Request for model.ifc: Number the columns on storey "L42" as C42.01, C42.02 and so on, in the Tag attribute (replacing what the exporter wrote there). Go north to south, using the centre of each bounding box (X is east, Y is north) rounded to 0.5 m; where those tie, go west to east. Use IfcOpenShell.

First a look at what the model holds.

```python
import ifcopenshell
import ifcopenshell.util.element
import ifcopenshell.util.placement

model = ifcopenshell.open("model.ifc")
print(model.schema)
storey = next(s for s in model.by_type("IfcBuildingStorey") if s.Name == "L42")
columns = [e for e in ifcopenshell.util.element.get_decomposition(storey) if e.is_a("IfcColumn")]
for e in sorted(columns, key=lambda e: e.id()):
    origin = ifcopenshell.util.placement.get_local_placement(e.ObjectPlacement)[:3, 3]
    print(e.id(), e.Tag, e.Name, origin.round(2) + 0.0, sep=" | ")
```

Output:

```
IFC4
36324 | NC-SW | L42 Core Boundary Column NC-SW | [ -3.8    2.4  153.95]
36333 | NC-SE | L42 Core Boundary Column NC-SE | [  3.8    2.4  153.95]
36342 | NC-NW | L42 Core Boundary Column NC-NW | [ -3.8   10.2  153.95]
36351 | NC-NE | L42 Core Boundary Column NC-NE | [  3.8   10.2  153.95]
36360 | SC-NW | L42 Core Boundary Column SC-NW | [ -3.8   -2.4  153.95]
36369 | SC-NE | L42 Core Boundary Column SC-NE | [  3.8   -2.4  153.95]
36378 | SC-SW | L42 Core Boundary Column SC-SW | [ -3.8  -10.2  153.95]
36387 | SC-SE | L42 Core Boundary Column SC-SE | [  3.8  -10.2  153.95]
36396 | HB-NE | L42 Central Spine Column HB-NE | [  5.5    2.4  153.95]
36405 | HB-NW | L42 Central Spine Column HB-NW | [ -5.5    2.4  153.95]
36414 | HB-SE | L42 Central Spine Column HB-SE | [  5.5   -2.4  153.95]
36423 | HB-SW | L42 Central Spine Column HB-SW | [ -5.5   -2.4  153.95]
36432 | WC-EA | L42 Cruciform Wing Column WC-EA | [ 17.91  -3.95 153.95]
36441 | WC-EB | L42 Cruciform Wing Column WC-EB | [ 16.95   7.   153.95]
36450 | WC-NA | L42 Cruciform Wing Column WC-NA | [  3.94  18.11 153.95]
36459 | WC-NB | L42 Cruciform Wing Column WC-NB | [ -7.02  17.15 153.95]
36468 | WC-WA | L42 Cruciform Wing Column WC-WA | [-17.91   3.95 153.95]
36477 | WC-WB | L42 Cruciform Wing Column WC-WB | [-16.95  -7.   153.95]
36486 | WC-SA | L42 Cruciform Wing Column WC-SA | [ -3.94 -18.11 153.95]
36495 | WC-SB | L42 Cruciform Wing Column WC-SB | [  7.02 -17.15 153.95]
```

```python
import ifcopenshell
import ifcopenshell.geom
import ifcopenshell.util.element
import ifcopenshell.util.shape

model = ifcopenshell.open("model.ifc")
settings = ifcopenshell.geom.settings()
settings.set("use-world-coords", True)


def centre(element):
    shape = ifcopenshell.geom.create_shape(settings, element)
    return ifcopenshell.util.shape.get_bbox_centroid(shape.geometry)


storey = next(s for s in model.by_type("IfcBuildingStorey") if s.Name == "L42")
columns = [e for e in ifcopenshell.util.element.get_decomposition(storey) if e.is_a("IfcColumn")]

# Insertion points can sit at a corner or the storey origin, so sort by the geometry (in metres).
centres = {e: centre(e) for e in columns}
columns.sort(key=lambda e: (-round(centres[e][1] / 0.5), centres[e][0]))

for i, e in enumerate(columns, start=1):
    number = f"C42.{i:02d}"
    e.Tag = number
    print(e.id(), number)

model.write("model_v2.ifc")
```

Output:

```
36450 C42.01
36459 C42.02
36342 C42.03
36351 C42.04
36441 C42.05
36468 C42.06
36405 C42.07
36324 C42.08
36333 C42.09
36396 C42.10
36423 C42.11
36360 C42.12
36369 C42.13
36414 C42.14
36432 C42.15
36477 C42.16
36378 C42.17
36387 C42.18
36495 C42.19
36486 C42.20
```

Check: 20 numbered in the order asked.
